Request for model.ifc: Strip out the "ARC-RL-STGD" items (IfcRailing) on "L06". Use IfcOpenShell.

First a look at what the model holds.

```python
import ifcopenshell
import ifcopenshell.util.element

model = ifcopenshell.open("model.ifc")
print(model.schema)
storey = next(s for s in model.by_type("IfcBuildingStorey") if s.Name == "L06")
railings = [e for e in ifcopenshell.util.element.get_decomposition(storey) if e.is_a("IfcRailing")]
seen = {}
for e in railings:
    element_type = ifcopenshell.util.element.get_type(e)
    name = element_type.Name if element_type not in (None, e) else None
    seen[name] = seen.get(name, 0) + 1
for name, count in sorted(seen.items(), key=str):
    print(count, "x", name)
```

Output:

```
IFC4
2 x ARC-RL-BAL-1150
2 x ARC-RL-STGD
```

```python
import ifcopenshell
import ifcopenshell.api.root
import ifcopenshell.util.element

model = ifcopenshell.open("model.ifc")

storey = next(s for s in model.by_type("IfcBuildingStorey") if s.Name == "L06")
railings = [e for e in ifcopenshell.util.element.get_decomposition(storey) if e.is_a("IfcRailing")]
targets = [e for e in railings if (t := ifcopenshell.util.element.get_type(e)) not in (None, e) and t.Name == "ARC-RL-STGD"]

for e in targets:
    ifcopenshell.api.root.remove_product(model, product=e)
print(len(targets), "removed")

model.write("model-out.ifc")
```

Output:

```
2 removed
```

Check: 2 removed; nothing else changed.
